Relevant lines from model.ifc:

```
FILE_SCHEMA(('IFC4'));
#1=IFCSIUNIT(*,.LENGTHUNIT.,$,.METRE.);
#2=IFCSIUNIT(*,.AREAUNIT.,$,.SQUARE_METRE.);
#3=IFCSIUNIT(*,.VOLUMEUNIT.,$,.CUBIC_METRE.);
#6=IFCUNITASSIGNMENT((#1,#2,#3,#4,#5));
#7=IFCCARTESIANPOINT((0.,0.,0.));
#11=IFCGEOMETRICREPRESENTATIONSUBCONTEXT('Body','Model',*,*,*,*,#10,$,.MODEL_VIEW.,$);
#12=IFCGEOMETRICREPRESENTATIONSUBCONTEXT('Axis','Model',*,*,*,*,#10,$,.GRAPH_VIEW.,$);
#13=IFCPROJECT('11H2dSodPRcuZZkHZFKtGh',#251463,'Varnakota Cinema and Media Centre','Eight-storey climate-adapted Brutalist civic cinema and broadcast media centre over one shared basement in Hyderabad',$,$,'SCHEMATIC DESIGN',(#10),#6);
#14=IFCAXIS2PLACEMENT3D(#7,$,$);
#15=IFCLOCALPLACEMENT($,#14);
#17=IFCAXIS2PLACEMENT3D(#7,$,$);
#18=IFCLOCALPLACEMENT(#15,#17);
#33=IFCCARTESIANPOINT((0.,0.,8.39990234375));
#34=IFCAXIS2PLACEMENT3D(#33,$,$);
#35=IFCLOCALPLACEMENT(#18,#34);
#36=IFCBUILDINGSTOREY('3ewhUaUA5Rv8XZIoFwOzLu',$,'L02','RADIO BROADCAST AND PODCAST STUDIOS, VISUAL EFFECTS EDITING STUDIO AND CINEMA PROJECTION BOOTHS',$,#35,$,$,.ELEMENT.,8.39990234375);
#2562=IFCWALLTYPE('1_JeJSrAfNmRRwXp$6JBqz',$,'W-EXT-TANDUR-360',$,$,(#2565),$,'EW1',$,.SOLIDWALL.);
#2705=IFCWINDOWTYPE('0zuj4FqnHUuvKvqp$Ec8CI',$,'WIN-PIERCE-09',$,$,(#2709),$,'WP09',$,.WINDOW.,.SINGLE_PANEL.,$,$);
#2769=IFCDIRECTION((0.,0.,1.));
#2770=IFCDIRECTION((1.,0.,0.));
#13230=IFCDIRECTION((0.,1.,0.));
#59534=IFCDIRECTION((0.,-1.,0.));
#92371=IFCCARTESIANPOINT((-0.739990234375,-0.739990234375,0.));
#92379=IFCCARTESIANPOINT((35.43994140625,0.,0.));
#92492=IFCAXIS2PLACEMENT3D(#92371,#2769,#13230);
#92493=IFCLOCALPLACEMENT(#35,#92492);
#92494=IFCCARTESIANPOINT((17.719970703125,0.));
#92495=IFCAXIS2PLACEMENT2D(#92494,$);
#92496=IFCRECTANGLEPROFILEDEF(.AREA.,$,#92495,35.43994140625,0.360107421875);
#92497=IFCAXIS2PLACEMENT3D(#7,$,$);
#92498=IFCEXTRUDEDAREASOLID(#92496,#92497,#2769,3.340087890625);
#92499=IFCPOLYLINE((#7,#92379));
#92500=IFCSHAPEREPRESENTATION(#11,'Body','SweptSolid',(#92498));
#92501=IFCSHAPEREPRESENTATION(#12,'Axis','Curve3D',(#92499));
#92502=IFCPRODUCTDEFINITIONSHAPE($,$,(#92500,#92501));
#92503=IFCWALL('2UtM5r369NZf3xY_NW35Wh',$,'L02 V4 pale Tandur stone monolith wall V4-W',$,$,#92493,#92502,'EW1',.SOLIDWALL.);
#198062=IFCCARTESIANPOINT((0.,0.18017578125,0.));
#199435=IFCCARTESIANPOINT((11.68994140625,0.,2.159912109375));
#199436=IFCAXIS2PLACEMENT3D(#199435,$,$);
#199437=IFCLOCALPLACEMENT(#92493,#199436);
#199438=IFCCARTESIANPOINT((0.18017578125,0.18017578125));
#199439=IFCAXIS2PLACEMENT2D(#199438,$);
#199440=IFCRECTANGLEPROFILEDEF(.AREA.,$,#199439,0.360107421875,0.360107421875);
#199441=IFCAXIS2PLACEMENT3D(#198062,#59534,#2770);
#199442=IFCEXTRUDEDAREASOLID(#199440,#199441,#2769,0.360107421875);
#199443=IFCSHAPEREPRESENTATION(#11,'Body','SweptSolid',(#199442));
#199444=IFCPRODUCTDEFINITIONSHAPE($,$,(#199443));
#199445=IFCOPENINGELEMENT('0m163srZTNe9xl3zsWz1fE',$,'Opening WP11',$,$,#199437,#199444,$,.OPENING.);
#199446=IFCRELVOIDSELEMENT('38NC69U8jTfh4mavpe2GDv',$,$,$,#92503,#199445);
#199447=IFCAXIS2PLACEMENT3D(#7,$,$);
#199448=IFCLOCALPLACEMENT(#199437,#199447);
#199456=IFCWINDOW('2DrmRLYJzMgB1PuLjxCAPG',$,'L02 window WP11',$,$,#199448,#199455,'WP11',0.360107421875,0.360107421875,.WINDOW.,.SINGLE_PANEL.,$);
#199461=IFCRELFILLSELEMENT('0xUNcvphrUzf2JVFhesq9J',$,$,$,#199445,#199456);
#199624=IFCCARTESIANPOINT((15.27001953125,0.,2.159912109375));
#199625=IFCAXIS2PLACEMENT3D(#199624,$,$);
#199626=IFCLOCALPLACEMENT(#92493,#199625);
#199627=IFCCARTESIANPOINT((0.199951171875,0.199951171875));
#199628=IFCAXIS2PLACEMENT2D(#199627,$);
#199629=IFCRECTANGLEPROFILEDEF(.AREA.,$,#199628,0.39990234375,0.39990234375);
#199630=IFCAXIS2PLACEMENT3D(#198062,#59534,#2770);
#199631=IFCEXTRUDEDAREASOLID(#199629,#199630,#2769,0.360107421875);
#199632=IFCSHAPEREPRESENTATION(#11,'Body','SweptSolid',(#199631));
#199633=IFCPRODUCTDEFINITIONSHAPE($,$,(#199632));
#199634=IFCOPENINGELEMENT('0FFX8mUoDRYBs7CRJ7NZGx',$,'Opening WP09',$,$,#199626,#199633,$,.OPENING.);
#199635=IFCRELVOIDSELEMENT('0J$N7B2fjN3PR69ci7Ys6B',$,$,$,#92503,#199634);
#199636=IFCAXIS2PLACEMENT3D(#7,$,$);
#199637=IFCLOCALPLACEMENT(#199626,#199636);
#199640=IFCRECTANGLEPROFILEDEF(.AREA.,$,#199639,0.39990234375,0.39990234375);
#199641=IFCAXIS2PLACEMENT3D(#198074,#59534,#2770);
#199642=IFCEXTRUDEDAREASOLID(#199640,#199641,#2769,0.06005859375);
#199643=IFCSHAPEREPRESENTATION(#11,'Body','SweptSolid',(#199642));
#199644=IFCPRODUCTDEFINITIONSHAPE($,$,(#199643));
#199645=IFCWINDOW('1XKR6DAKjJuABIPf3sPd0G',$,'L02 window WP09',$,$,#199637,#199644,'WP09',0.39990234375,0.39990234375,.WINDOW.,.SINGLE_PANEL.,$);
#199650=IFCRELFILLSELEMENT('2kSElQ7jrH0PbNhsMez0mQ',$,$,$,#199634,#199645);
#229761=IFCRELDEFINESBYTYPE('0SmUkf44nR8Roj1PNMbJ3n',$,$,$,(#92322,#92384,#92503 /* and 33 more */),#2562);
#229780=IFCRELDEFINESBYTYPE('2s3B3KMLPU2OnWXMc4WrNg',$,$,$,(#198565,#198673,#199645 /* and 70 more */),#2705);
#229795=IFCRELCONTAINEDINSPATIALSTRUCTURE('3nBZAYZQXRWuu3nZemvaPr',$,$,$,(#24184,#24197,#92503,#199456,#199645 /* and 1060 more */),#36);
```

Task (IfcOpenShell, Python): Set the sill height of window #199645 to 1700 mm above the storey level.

```python
import numpy as np
import ifcopenshell
import ifcopenshell.api.geometry
import ifcopenshell.geom
import ifcopenshell.util.element
import ifcopenshell.util.placement
import ifcopenshell.util.shape
import ifcopenshell.util.unit

model = ifcopenshell.open("model.ifc")
unit_scale = ifcopenshell.util.unit.calculate_unit_scale(model)

window = model.by_id(199645)
opening = window.FillsVoids[0].RelatingOpeningElement
storey = ifcopenshell.util.element.get_container(window, ifc_class="IfcBuildingStorey")
level = ifcopenshell.util.placement.get_local_placement(storey.ObjectPlacement)[2, 3]

# The opening's origin need not be at the sill, so measure its lowest point.
shape = ifcopenshell.geom.create_shape(ifcopenshell.geom.settings(), opening)
bottom = ifcopenshell.util.shape.get_shape_bottom_elevation(shape, shape.geometry) / unit_scale
dz = level + 1.7 / unit_scale - bottom

shift = np.array([0.0, 0.0, dz])
# The window is placed relative to its opening, so it follows when the opening moves.
matrix = ifcopenshell.util.placement.get_local_placement(opening.ObjectPlacement)
matrix[:3, 3] += shift
ifcopenshell.api.geometry.edit_object_placement(
    model, product=opening, matrix=matrix, is_si=False, should_transform_children=True
)

print(f"moved by {dz * unit_scale:+.3f} m")

model.write("model_v2.ifc")
```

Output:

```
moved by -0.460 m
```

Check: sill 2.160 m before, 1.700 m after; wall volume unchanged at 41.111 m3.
